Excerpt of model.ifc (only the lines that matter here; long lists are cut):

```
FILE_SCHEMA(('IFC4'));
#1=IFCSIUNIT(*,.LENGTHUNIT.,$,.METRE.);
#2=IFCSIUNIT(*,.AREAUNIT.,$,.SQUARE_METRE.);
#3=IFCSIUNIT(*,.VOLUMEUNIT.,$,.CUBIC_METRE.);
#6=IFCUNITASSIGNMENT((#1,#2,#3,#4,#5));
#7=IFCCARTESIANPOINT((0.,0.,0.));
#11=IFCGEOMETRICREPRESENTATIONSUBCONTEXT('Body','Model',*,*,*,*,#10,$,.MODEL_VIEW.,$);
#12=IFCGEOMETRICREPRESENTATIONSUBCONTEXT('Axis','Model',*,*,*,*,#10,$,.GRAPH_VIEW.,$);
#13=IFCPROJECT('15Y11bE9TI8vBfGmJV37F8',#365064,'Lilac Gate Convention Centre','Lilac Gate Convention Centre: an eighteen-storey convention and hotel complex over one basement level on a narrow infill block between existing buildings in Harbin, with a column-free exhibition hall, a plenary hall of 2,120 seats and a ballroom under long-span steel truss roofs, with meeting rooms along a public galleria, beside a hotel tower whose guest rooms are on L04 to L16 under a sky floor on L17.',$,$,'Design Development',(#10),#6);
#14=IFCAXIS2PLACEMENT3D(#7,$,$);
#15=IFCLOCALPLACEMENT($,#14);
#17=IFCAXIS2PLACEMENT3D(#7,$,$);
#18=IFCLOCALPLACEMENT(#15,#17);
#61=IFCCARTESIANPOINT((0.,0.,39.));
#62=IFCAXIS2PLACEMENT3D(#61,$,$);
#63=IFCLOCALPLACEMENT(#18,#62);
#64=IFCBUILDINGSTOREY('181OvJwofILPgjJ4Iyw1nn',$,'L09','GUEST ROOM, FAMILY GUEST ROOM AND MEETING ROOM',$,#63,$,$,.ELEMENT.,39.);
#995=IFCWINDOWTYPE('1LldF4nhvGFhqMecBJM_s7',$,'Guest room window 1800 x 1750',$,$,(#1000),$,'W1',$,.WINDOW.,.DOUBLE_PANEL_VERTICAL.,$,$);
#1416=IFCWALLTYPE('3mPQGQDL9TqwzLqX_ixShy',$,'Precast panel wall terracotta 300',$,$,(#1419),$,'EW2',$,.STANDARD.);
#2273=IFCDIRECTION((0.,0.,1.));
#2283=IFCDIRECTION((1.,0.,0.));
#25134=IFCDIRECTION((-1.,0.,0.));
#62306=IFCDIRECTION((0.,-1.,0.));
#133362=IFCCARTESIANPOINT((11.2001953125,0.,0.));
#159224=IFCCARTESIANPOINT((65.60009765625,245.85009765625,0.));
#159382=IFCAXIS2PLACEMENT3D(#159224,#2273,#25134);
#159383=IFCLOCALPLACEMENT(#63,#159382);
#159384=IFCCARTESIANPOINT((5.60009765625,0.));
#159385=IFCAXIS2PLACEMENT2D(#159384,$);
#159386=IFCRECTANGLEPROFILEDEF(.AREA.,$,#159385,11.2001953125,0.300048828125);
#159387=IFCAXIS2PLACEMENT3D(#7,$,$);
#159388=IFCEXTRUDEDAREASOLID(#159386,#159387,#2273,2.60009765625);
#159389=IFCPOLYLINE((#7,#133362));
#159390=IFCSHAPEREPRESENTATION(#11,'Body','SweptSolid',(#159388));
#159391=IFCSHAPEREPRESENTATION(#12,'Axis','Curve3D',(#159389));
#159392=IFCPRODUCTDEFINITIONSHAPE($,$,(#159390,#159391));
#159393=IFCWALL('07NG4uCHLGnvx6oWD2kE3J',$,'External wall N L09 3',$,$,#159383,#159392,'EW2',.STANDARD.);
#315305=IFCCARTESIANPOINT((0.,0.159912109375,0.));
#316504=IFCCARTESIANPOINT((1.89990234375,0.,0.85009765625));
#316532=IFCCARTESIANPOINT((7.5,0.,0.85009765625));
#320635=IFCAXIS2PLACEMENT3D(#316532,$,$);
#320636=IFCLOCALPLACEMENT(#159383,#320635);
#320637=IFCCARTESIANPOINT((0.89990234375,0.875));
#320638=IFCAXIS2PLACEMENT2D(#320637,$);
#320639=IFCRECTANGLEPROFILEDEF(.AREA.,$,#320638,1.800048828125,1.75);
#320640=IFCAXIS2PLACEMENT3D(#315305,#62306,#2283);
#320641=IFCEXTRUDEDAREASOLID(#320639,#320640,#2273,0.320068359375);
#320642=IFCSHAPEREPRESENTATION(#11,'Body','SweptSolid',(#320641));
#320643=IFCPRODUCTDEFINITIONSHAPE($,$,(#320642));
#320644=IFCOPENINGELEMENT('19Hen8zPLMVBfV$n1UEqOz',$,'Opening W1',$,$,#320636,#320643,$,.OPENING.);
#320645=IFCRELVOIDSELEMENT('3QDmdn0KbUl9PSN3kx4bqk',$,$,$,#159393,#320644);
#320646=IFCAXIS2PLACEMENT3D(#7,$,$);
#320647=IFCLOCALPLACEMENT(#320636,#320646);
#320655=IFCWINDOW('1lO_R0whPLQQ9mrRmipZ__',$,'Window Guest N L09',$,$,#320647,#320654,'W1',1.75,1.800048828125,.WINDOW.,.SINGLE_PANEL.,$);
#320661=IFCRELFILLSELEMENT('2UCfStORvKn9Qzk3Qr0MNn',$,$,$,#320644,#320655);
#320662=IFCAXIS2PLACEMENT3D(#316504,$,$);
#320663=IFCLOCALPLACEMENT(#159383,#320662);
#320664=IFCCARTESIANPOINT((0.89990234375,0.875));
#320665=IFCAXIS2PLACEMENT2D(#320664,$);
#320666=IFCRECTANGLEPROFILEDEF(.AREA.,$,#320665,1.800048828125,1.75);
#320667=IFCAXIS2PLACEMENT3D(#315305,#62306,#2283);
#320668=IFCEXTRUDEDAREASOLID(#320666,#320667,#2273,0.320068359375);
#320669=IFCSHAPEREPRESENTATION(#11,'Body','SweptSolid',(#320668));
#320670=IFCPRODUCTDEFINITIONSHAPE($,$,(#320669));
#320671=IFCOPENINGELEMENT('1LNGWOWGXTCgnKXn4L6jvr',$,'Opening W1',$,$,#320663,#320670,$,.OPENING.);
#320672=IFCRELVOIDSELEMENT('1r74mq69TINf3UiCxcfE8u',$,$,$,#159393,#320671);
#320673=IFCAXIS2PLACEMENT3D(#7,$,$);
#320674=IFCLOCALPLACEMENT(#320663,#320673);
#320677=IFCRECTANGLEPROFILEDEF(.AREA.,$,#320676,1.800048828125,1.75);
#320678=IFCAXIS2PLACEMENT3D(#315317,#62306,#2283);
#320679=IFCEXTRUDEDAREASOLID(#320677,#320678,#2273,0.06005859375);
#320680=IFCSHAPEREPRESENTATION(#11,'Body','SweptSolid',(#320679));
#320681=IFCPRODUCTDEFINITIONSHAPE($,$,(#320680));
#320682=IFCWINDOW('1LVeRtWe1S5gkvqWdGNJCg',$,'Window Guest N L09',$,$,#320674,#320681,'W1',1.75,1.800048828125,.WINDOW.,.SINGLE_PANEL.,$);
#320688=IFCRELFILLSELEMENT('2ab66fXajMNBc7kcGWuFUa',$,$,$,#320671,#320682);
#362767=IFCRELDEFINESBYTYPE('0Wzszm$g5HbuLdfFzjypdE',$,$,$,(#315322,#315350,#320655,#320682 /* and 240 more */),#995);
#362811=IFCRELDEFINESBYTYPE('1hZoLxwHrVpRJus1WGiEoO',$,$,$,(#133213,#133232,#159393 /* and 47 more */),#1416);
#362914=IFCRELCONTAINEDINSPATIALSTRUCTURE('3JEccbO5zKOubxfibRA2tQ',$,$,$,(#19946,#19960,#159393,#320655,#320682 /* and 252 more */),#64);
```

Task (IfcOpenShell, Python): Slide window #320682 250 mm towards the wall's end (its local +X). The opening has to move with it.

```python
import ifcopenshell
import ifcopenshell.api.geometry
import ifcopenshell.util.placement
import ifcopenshell.util.unit

model = ifcopenshell.open("model.ifc")
unit_scale = ifcopenshell.util.unit.calculate_unit_scale(model)

window = model.by_guid("1LVeRtWe1S5gkvqWdGNJCg")
opening = window.FillsVoids[0].RelatingOpeningElement
wall = opening.VoidsElements[0].RelatingBuildingElement

wall_matrix = ifcopenshell.util.placement.get_local_placement(wall.ObjectPlacement)
shift = wall_matrix[:3, 0] * 0.25 / unit_scale
before = ifcopenshell.util.placement.get_local_placement(window.ObjectPlacement)[:3, 3].copy()

# The window is placed relative to its opening, so it follows when the opening moves.
matrix = ifcopenshell.util.placement.get_local_placement(opening.ObjectPlacement)
matrix[:3, 3] += shift
ifcopenshell.api.geometry.edit_object_placement(
    model, product=opening, matrix=matrix, is_si=False, should_transform_children=True
)

after = ifcopenshell.util.placement.get_local_placement(window.ObjectPlacement)[:3, 3]
print("window moved by", (after - before).round(3) + 0.0)

model.write("model_edited.ifc")
```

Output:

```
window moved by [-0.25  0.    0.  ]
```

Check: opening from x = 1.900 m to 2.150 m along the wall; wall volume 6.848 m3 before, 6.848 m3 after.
